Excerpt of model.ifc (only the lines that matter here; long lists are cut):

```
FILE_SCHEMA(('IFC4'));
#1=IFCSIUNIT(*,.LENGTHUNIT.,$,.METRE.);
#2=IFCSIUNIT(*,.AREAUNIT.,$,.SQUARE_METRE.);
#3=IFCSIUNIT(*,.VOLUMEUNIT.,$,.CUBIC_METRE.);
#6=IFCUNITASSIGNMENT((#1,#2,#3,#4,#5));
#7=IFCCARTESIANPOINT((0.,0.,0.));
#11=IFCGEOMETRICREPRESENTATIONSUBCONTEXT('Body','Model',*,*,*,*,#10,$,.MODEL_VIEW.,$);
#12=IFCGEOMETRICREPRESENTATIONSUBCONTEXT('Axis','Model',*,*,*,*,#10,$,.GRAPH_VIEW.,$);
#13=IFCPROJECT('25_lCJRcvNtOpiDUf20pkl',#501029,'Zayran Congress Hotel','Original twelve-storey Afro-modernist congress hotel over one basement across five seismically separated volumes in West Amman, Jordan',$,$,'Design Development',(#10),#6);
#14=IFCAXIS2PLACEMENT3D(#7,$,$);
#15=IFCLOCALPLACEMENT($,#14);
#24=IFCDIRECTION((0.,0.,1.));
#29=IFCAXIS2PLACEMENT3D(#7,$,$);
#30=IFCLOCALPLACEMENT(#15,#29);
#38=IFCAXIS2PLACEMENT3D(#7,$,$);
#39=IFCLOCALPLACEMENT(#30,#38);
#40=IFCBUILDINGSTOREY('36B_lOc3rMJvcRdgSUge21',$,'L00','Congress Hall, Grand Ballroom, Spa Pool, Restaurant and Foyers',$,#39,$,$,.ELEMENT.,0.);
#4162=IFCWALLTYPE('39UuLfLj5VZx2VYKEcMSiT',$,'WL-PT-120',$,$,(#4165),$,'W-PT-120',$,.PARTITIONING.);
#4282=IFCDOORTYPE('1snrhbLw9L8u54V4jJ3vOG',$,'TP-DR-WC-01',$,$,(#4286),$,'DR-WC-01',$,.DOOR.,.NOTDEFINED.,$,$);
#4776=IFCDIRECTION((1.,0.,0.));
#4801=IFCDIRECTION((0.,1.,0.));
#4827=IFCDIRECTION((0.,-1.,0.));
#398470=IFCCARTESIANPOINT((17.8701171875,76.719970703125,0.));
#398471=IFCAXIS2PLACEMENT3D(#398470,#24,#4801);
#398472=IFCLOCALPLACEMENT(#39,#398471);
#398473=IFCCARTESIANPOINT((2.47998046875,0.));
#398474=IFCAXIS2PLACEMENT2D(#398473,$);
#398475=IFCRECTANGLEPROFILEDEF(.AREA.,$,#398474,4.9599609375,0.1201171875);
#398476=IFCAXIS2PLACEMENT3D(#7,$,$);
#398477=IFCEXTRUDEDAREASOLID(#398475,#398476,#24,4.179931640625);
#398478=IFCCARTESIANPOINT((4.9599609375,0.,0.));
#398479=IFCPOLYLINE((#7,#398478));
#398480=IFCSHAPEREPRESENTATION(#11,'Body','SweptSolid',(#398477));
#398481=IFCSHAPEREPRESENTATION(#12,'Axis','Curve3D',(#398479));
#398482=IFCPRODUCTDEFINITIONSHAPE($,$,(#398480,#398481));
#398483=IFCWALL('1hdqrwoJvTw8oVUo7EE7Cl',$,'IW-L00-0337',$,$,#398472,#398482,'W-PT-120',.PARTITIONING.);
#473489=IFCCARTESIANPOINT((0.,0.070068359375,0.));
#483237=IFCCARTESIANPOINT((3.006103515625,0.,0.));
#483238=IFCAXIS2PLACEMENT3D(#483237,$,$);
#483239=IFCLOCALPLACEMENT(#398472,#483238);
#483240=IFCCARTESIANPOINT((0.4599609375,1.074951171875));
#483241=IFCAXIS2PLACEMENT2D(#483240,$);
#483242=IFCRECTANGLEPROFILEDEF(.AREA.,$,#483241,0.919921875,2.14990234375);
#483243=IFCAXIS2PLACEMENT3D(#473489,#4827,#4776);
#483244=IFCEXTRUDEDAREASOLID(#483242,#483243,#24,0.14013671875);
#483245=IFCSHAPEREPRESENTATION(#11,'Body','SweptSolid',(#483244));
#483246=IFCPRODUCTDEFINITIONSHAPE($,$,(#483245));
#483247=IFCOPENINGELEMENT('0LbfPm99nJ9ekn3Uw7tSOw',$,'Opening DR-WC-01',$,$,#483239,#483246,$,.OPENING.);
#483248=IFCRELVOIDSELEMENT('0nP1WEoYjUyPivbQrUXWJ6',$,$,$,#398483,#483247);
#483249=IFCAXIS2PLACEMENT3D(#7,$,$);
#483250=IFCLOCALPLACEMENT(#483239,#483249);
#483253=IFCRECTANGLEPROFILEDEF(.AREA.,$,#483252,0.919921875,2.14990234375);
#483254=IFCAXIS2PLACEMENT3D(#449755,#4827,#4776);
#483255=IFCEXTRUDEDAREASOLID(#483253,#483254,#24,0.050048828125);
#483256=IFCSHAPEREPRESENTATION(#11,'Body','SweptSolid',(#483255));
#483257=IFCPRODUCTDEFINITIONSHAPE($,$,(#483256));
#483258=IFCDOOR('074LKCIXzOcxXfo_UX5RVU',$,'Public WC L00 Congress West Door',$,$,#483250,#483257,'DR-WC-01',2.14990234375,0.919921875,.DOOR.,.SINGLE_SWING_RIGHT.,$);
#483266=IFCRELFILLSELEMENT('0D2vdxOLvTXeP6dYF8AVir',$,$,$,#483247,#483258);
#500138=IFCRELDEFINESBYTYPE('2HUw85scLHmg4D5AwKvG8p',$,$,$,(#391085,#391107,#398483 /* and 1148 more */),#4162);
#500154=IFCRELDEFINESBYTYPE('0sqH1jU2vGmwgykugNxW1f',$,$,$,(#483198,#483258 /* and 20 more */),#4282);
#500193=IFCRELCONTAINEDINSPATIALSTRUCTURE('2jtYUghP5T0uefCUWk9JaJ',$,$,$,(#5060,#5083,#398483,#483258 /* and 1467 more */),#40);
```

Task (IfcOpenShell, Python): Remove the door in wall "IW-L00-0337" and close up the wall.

```python
import ifcopenshell
import ifcopenshell.api.feature
import ifcopenshell.api.root
import ifcopenshell.geom
import ifcopenshell.util.shape

model = ifcopenshell.open("model.ifc")
settings = ifcopenshell.geom.settings()


def volume(element):
    """Net volume in cubic metres, openings subtracted."""
    shape = ifcopenshell.geom.create_shape(settings, element)
    return ifcopenshell.util.shape.get_volume(shape.geometry)


door = model.by_guid("074LKCIXzOcxXfo_UX5RVU")
opening = door.FillsVoids[0].RelatingOpeningElement
wall = opening.VoidsElements[0].RelatingBuildingElement
before = volume(wall)

ifcopenshell.api.root.remove_product(model, product=door)
ifcopenshell.api.feature.remove_feature(model, feature=opening)

after = volume(wall)

print(f"wall volume {before:.3f} -> {after:.3f} m3")

model.write("model_v2.ifc")
```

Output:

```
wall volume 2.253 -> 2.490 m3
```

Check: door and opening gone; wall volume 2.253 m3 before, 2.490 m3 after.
